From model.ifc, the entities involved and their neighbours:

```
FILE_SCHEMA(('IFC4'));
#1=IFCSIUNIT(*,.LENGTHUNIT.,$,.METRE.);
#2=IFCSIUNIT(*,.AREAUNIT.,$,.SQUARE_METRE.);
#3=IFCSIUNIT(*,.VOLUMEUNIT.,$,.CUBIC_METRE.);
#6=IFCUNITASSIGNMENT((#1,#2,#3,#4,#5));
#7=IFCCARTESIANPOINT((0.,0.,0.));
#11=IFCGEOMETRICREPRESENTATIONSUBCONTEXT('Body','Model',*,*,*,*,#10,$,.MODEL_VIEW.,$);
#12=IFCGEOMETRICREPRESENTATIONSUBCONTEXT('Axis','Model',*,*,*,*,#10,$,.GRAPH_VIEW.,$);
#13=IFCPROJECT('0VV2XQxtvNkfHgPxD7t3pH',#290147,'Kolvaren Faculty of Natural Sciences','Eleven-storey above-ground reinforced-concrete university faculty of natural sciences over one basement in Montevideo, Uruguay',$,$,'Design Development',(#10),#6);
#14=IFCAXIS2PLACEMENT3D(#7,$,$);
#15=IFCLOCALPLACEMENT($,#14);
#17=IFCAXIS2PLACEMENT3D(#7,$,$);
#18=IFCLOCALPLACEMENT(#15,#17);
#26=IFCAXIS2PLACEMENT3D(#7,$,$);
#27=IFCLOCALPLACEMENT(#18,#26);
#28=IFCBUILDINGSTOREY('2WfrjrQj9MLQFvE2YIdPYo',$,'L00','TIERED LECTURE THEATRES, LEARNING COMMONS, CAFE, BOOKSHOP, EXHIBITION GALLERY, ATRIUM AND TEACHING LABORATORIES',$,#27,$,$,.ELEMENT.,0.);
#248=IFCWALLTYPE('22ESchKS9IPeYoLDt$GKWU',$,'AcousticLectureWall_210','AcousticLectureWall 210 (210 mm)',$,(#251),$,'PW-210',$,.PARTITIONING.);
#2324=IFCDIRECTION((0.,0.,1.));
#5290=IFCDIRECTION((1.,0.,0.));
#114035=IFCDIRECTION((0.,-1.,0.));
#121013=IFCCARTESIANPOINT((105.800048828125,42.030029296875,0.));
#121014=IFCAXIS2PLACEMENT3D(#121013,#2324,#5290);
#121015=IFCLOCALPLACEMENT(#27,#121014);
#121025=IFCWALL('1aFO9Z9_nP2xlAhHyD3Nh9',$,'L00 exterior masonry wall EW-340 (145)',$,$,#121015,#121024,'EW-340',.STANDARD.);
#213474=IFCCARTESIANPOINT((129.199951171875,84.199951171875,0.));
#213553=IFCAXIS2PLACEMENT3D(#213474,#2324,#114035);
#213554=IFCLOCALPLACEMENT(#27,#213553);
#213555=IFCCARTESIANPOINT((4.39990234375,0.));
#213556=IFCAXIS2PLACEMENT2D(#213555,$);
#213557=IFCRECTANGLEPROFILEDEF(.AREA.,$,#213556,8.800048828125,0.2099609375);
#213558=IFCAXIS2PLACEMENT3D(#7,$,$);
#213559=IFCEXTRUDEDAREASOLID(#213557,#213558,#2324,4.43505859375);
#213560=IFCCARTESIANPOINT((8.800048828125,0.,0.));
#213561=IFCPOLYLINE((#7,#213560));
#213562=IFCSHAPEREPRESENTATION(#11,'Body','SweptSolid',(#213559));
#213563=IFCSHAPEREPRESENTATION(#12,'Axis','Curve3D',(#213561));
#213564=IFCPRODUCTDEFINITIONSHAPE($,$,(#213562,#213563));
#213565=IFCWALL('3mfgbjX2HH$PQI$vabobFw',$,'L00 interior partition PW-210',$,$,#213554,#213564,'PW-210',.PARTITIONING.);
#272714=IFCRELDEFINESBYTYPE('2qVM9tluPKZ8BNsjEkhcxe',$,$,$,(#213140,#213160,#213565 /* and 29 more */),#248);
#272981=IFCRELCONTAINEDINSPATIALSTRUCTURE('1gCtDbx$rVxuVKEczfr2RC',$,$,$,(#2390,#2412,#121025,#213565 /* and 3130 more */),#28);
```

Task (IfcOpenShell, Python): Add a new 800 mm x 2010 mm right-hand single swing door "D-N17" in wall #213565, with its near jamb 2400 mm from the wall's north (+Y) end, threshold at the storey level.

```python
import numpy as np
import ifcopenshell
import ifcopenshell.api.feature
import ifcopenshell.api.geometry
import ifcopenshell.api.root
import ifcopenshell.api.spatial
import ifcopenshell.geom
import ifcopenshell.util.element
import ifcopenshell.util.placement
import ifcopenshell.util.representation
import ifcopenshell.util.shape
import ifcopenshell.util.unit

model = ifcopenshell.open("model.ifc")
unit_scale = ifcopenshell.util.unit.calculate_unit_scale(model)
settings = ifcopenshell.geom.settings()


def volume(element):
    """Net volume in cubic metres, openings subtracted."""
    shape = ifcopenshell.geom.create_shape(settings, element)
    return ifcopenshell.util.shape.get_volume(shape.geometry)


wall = model.by_guid("3mfgbjX2HH$PQI$vabobFw")
storey = ifcopenshell.util.element.get_container(wall, ifc_class="IfcBuildingStorey")
context = ifcopenshell.util.representation.get_context(model, "Model", "Body", "MODEL_VIEW")
before = volume(wall)

width, height, from_end, sill = 0.8, 2.01, 2.4, 0.0  # metres

# The wall runs along its own X axis, and the end named is its -X end.
wall_shape = ifcopenshell.geom.create_shape(settings, wall)
x, y, z = ifcopenshell.util.shape.get_vertices(wall_shape.geometry).T
start = x.min() + from_end
face, thickness = float(y.min()), float(y.max() - y.min())
wall_matrix = ifcopenshell.util.placement.get_local_placement(wall.ObjectPlacement)
level = ifcopenshell.util.placement.get_local_placement(storey.ObjectPlacement)[2, 3]


def in_wall(x, y):
    """Placement at x, y metres in the wall's axes, at sill height."""
    matrix = wall_matrix.copy()
    matrix[:, 3] = wall_matrix @ np.array([x / unit_scale, y / unit_scale, 0.0, 1.0])
    matrix[2, 3] = level + sill / unit_scale
    return matrix


# Opening: a box that overshoots both wall faces by 50 mm.
opening = ifcopenshell.api.root.create_entity(model, ifc_class="IfcOpeningElement", predefined_type="OPENING")
box = ifcopenshell.api.geometry.add_wall_representation(
    model, context=context, length=width, height=height, thickness=thickness + 0.1
)
ifcopenshell.api.geometry.assign_representation(model, product=opening, representation=box)
ifcopenshell.api.geometry.edit_object_placement(model, product=opening, matrix=in_wall(start, face - 0.05), is_si=False)
ifcopenshell.api.feature.add_feature(model, feature=opening, element=wall)

door = ifcopenshell.api.root.create_entity(model, ifc_class="IfcDoor", name="D-N17", predefined_type="DOOR")
door.OverallWidth, door.OverallHeight = width / unit_scale, height / unit_scale
door.OperationType = "SINGLE_SWING_RIGHT"
body = ifcopenshell.api.geometry.add_door_representation(
    model,
    context=context,
    overall_width=door.OverallWidth,
    overall_height=door.OverallHeight,
    operation_type="SINGLE_SWING_RIGHT",
    lining_properties={"LiningDepth": thickness / unit_scale, "ThresholdDepth": thickness / unit_scale},
)
ifcopenshell.api.geometry.assign_representation(model, product=door, representation=body)
ifcopenshell.api.spatial.assign_container(model, products=[door], relating_structure=storey)
ifcopenshell.api.feature.add_filling(model, opening=opening, element=door)

# The lining spans the wall, so the door starts at the wall face.
ifcopenshell.api.geometry.edit_object_placement(model, product=door, matrix=in_wall(start, face), is_si=False)

after = volume(wall)

print(f"wall volume {before:.3f} -> {after:.3f} m3")

model.write("model_rev.ifc")
```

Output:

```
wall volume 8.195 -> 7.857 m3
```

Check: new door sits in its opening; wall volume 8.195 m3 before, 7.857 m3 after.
